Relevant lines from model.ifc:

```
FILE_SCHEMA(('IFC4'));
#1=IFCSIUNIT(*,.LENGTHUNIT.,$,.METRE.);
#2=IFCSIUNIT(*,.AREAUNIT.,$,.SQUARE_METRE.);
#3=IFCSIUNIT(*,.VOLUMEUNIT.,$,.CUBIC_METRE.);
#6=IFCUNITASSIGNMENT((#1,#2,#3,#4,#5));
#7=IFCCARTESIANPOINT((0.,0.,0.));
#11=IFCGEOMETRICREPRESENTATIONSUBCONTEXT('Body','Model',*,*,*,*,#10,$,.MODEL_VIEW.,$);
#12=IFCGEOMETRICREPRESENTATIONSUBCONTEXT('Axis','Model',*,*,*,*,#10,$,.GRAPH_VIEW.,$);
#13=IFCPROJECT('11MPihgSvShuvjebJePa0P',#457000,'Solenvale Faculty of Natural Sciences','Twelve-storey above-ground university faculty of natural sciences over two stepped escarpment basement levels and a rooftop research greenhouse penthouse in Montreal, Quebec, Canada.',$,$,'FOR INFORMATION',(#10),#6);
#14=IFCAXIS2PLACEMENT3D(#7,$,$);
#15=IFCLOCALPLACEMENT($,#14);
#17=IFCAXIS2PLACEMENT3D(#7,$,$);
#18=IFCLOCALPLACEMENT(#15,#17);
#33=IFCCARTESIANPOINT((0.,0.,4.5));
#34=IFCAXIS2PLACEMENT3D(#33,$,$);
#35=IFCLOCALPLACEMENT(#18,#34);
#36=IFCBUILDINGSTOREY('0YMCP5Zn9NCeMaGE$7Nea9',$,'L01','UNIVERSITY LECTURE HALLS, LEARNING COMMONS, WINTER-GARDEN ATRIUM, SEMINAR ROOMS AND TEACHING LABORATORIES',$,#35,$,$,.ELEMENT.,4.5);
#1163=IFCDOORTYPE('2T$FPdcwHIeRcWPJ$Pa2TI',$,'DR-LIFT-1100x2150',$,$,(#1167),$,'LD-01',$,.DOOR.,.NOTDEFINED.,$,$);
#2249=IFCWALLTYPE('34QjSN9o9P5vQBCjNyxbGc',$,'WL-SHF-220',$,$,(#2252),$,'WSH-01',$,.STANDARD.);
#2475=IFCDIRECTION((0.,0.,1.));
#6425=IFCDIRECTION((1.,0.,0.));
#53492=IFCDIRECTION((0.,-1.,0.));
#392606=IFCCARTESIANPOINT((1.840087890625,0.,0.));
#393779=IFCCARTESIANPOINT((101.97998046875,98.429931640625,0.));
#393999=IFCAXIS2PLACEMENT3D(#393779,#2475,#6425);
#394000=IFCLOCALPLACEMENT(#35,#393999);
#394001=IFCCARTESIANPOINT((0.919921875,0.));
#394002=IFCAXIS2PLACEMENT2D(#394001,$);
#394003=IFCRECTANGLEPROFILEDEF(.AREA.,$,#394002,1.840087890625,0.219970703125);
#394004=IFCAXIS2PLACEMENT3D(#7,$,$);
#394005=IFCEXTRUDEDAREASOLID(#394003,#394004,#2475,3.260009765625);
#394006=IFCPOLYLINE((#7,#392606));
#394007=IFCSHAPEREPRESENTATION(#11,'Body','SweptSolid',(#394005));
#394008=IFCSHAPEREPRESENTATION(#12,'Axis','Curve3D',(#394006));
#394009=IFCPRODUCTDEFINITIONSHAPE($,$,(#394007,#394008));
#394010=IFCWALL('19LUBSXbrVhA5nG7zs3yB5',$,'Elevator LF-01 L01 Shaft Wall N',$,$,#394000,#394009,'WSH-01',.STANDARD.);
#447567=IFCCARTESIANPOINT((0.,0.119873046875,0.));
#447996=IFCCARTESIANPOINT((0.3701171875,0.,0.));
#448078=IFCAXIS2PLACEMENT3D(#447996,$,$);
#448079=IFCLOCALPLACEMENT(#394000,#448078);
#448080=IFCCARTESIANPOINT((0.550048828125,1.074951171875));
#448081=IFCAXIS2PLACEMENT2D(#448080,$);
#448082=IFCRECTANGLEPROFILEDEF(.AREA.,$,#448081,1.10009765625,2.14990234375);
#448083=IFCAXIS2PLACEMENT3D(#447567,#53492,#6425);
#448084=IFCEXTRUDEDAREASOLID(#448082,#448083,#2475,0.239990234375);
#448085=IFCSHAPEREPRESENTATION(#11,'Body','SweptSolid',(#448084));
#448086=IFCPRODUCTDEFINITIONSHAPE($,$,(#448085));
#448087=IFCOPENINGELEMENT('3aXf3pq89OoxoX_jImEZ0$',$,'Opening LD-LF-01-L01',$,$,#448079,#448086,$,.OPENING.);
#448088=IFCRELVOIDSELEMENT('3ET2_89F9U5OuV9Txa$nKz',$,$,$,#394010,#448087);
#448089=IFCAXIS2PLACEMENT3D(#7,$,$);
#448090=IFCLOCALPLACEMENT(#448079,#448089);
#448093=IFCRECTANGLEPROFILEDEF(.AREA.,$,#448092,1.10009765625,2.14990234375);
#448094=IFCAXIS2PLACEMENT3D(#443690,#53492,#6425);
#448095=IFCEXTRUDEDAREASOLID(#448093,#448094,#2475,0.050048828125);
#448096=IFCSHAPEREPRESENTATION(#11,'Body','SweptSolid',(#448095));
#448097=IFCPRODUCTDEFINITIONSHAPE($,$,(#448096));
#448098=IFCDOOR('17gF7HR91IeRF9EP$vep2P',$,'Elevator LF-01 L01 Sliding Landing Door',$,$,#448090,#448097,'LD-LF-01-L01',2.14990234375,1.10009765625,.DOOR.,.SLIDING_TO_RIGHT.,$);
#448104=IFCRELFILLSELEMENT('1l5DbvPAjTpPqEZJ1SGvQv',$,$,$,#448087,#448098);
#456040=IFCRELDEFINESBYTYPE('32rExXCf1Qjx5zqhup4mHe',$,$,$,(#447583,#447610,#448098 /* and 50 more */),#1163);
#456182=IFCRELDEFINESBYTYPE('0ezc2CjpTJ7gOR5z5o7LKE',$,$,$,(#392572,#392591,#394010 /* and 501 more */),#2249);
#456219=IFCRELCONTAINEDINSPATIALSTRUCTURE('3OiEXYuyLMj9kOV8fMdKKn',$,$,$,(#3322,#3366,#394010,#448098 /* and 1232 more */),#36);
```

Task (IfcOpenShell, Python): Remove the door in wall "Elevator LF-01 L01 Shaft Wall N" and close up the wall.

```python
import ifcopenshell
import ifcopenshell.api.feature
import ifcopenshell.api.root
import ifcopenshell.geom
import ifcopenshell.util.shape

model = ifcopenshell.open("model.ifc")
settings = ifcopenshell.geom.settings()


def volume(element):
    """Net volume in cubic metres, openings subtracted."""
    shape = ifcopenshell.geom.create_shape(settings, element)
    return ifcopenshell.util.shape.get_volume(shape.geometry)


door = model.by_id(448098)
opening = door.FillsVoids[0].RelatingOpeningElement
wall = opening.VoidsElements[0].RelatingBuildingElement
before = volume(wall)

ifcopenshell.api.root.remove_product(model, product=door)
ifcopenshell.api.feature.remove_feature(model, feature=opening)

after = volume(wall)

print(f"wall volume {before:.3f} -> {after:.3f} m3")

model.write("model_updated.ifc")
```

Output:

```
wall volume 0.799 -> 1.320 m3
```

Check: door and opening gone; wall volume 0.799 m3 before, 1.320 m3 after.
